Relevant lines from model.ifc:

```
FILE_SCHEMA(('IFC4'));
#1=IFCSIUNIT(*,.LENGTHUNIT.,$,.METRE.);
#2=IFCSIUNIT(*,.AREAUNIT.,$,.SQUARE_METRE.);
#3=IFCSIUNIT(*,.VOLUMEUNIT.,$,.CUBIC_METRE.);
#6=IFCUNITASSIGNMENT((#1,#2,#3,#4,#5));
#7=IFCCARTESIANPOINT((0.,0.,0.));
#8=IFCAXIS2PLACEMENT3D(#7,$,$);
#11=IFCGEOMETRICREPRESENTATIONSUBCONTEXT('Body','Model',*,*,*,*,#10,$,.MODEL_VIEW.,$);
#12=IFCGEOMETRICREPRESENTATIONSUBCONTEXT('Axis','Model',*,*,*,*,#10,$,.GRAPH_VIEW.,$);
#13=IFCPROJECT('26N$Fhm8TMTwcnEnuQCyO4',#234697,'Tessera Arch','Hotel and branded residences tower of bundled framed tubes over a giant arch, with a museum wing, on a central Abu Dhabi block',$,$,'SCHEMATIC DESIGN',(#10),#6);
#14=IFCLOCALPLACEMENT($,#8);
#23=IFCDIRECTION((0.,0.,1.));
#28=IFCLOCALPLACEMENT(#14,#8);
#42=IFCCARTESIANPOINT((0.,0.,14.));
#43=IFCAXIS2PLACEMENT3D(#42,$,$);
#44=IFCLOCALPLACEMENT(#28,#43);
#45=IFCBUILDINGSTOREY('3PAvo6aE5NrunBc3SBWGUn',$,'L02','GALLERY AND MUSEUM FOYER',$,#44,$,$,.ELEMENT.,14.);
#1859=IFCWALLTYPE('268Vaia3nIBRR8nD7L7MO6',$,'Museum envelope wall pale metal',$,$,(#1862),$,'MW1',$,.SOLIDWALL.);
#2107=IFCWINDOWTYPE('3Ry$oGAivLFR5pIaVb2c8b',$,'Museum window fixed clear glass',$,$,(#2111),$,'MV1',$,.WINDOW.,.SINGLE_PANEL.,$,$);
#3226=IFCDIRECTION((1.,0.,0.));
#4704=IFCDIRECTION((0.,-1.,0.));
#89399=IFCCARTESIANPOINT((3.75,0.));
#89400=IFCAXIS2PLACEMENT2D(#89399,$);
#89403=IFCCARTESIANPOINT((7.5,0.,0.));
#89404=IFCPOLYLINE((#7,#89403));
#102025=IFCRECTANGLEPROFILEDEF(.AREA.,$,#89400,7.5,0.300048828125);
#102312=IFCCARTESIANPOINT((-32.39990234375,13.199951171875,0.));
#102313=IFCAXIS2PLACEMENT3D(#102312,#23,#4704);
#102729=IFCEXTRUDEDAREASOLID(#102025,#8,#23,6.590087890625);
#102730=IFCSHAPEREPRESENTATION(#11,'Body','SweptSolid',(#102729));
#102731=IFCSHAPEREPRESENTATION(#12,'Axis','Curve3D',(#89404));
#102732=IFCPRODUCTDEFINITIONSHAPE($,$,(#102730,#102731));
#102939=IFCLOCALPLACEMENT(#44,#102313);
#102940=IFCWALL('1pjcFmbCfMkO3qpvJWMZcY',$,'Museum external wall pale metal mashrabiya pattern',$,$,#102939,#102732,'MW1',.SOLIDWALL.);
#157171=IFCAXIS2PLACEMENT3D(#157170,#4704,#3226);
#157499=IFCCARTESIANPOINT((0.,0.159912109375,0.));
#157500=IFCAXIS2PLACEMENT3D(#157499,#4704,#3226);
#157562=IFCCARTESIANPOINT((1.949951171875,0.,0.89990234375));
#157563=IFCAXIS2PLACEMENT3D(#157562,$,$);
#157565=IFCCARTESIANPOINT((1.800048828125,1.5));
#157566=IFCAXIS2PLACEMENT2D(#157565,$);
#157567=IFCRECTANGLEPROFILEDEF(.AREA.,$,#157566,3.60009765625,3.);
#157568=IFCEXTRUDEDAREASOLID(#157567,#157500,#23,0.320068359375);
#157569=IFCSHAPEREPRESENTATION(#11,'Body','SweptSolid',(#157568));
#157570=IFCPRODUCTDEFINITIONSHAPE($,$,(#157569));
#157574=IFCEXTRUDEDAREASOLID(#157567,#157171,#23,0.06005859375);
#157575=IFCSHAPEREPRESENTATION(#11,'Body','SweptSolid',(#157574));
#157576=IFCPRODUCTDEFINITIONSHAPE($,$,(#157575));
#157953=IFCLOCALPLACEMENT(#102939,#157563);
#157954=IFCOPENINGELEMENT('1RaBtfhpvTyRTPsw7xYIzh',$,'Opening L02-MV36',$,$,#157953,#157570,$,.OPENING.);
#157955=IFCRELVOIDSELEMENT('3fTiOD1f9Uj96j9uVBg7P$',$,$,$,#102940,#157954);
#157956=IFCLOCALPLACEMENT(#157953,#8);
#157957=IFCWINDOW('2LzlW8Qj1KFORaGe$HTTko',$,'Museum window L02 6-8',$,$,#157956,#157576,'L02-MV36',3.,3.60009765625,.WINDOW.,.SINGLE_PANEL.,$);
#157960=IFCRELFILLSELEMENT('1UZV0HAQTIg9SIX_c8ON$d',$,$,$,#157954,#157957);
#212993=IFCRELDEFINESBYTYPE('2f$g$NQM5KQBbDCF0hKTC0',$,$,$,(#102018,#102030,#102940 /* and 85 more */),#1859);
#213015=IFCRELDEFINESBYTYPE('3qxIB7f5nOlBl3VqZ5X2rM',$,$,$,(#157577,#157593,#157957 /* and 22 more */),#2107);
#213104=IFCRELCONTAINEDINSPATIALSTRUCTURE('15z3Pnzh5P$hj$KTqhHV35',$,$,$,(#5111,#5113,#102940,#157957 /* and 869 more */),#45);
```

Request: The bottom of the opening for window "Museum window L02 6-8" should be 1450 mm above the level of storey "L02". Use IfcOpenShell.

```python
import numpy as np
import ifcopenshell
import ifcopenshell.api.geometry
import ifcopenshell.geom
import ifcopenshell.util.element
import ifcopenshell.util.placement
import ifcopenshell.util.shape
import ifcopenshell.util.unit

model = ifcopenshell.open("model.ifc")
unit_scale = ifcopenshell.util.unit.calculate_unit_scale(model)

window = model.by_guid("2LzlW8Qj1KFORaGe$HTTko")
opening = window.FillsVoids[0].RelatingOpeningElement
storey = ifcopenshell.util.element.get_container(window, ifc_class="IfcBuildingStorey")
level = ifcopenshell.util.placement.get_local_placement(storey.ObjectPlacement)[2, 3]

# The opening's origin need not be at the sill, so measure its lowest point.
shape = ifcopenshell.geom.create_shape(ifcopenshell.geom.settings(), opening)
bottom = ifcopenshell.util.shape.get_shape_bottom_elevation(shape, shape.geometry) / unit_scale
dz = level + 1.45 / unit_scale - bottom

shift = np.array([0.0, 0.0, dz])
# The window is placed relative to its opening, so it follows when the opening moves.
matrix = ifcopenshell.util.placement.get_local_placement(opening.ObjectPlacement)
matrix[:3, 3] += shift
ifcopenshell.api.geometry.edit_object_placement(
    model, product=opening, matrix=matrix, is_si=False, should_transform_children=True
)

print(f"moved by {dz * unit_scale:+.3f} m")

model.write("model_edited.ifc")
```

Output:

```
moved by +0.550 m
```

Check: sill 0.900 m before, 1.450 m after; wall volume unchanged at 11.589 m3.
